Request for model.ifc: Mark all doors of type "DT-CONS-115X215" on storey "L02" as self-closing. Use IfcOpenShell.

First a look at what the model holds.

```python
import ifcopenshell
import ifcopenshell.util.element

model = ifcopenshell.open("model.ifc")
print(model.schema)
storey = next(s for s in model.by_type("IfcBuildingStorey") if s.Name == "L02")
doors = [e for e in ifcopenshell.util.element.get_decomposition(storey) if e.is_a("IfcDoor")]
seen = {}
for e in doors:
    element_type = ifcopenshell.util.element.get_type(e)
    key = (element_type.Name if element_type != e and element_type else None, ifcopenshell.util.element.get_pset(e, "Pset_DoorCommon", "SelfClosing"))
    seen[key] = seen.get(key, 0) + 1
for (name, value), count in sorted(seen.items(), key=str):
    print(count, "x", name, "|", value)
```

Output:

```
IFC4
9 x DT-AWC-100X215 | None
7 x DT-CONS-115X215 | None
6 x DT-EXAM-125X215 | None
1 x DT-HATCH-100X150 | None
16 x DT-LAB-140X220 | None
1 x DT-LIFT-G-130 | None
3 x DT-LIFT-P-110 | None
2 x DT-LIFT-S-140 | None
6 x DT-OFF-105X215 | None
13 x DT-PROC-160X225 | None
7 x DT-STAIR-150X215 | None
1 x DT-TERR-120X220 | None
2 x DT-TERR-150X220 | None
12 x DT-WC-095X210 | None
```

```python
import ifcopenshell
import ifcopenshell.api.pset
import ifcopenshell.util.element

model = ifcopenshell.open("model.ifc")

storey = next(s for s in model.by_type("IfcBuildingStorey") if s.Name == "L02")
doors = [e for e in ifcopenshell.util.element.get_decomposition(storey) if e.is_a("IfcDoor")]

count = 0
for e in doors:
    element_type = ifcopenshell.util.element.get_type(e)
    if element_type in (None, e) or element_type.Name != "DT-CONS-115X215":
        continue
    # add_pset returns the element's existing set when there is one.
    pset = ifcopenshell.api.pset.add_pset(model, product=e, name="Pset_DoorCommon")
    ifcopenshell.api.pset.edit_pset(model, pset=pset, properties={"SelfClosing": True})
    count += 1

print(count, "doors updated")

model.write("model-out.ifc")
```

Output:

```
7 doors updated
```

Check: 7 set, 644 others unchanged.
